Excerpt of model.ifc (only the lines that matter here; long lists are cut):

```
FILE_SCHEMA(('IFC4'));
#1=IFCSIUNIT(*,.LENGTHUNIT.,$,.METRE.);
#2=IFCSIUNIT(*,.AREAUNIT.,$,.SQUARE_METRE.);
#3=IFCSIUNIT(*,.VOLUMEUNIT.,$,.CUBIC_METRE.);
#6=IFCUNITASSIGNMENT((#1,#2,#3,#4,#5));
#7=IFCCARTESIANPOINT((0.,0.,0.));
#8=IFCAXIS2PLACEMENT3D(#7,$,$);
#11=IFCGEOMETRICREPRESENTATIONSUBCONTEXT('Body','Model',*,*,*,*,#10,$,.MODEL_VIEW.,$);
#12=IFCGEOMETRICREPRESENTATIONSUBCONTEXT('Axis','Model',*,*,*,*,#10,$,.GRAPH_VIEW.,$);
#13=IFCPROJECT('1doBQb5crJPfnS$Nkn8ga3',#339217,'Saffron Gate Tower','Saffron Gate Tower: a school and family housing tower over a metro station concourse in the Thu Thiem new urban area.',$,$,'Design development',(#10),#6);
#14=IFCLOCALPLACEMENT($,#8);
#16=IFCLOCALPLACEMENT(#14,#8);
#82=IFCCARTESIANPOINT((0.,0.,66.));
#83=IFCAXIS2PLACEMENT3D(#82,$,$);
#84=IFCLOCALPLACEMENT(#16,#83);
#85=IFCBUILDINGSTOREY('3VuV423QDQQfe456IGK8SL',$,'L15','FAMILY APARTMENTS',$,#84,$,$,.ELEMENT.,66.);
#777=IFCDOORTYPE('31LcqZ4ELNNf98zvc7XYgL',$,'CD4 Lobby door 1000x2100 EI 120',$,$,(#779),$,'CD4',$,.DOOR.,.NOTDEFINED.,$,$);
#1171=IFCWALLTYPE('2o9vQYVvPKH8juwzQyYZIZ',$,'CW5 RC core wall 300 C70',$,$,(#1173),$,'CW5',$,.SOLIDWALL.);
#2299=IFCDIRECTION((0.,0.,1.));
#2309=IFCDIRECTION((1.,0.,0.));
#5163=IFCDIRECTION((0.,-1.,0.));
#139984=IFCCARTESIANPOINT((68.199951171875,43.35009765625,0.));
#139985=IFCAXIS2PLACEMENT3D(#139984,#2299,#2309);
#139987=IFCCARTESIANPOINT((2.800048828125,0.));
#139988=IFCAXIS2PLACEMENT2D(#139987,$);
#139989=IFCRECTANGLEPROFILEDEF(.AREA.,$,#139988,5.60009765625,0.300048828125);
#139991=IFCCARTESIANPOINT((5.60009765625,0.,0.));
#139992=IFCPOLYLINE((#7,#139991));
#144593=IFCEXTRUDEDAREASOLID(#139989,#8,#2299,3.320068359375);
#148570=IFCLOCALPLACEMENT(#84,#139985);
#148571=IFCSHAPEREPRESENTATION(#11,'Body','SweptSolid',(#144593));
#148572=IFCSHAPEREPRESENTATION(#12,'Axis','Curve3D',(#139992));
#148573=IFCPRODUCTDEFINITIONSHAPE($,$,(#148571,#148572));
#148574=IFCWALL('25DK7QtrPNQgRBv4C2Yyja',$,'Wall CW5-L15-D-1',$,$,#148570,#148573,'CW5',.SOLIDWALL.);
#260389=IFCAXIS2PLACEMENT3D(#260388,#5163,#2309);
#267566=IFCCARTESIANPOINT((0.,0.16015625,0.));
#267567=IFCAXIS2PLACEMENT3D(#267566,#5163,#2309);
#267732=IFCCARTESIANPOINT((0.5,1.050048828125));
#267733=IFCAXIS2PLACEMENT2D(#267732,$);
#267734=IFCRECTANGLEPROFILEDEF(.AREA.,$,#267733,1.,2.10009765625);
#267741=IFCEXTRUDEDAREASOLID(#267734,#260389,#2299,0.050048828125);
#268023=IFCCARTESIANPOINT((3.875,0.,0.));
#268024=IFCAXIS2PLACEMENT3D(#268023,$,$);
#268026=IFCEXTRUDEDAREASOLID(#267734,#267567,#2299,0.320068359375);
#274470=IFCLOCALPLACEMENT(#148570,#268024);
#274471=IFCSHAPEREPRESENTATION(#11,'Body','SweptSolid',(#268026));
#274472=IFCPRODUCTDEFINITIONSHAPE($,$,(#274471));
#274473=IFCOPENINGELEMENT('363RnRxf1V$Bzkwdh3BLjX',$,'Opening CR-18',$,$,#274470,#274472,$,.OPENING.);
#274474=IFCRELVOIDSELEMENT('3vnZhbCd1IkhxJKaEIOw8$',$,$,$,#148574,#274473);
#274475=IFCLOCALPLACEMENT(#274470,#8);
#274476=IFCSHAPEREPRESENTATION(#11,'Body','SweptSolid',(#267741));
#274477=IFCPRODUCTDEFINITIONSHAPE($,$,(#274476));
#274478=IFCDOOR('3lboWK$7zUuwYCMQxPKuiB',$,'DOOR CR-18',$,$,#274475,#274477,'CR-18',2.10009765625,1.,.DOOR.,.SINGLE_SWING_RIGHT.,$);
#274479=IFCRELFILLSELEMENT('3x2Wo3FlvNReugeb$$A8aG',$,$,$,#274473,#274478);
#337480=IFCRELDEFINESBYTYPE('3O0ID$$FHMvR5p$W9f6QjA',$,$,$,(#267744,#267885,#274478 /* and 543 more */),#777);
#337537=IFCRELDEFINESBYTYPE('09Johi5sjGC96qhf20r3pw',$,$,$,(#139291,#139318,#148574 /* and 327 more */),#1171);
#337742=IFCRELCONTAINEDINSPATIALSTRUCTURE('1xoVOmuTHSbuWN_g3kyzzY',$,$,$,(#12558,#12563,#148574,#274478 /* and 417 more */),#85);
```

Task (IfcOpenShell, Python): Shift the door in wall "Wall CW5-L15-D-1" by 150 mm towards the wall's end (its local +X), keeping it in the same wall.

```python
import ifcopenshell
import ifcopenshell.api.geometry
import ifcopenshell.util.placement
import ifcopenshell.util.unit

model = ifcopenshell.open("model.ifc")
unit_scale = ifcopenshell.util.unit.calculate_unit_scale(model)

door = model.by_guid("3lboWK$7zUuwYCMQxPKuiB")
opening = door.FillsVoids[0].RelatingOpeningElement
wall = opening.VoidsElements[0].RelatingBuildingElement

wall_matrix = ifcopenshell.util.placement.get_local_placement(wall.ObjectPlacement)
shift = wall_matrix[:3, 0] * 0.15 / unit_scale
before = ifcopenshell.util.placement.get_local_placement(door.ObjectPlacement)[:3, 3].copy()

# The door is placed relative to its opening, so it follows when the opening moves.
matrix = ifcopenshell.util.placement.get_local_placement(opening.ObjectPlacement)
matrix[:3, 3] += shift
ifcopenshell.api.geometry.edit_object_placement(
    model, product=opening, matrix=matrix, is_si=False, should_transform_children=True
)

after = ifcopenshell.util.placement.get_local_placement(door.ObjectPlacement)[:3, 3]
print("door moved by", (after - before).round(3) + 0.0)

model.write("model_edited.ifc")
```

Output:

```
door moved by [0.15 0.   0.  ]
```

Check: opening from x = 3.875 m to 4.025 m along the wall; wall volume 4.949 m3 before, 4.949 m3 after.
